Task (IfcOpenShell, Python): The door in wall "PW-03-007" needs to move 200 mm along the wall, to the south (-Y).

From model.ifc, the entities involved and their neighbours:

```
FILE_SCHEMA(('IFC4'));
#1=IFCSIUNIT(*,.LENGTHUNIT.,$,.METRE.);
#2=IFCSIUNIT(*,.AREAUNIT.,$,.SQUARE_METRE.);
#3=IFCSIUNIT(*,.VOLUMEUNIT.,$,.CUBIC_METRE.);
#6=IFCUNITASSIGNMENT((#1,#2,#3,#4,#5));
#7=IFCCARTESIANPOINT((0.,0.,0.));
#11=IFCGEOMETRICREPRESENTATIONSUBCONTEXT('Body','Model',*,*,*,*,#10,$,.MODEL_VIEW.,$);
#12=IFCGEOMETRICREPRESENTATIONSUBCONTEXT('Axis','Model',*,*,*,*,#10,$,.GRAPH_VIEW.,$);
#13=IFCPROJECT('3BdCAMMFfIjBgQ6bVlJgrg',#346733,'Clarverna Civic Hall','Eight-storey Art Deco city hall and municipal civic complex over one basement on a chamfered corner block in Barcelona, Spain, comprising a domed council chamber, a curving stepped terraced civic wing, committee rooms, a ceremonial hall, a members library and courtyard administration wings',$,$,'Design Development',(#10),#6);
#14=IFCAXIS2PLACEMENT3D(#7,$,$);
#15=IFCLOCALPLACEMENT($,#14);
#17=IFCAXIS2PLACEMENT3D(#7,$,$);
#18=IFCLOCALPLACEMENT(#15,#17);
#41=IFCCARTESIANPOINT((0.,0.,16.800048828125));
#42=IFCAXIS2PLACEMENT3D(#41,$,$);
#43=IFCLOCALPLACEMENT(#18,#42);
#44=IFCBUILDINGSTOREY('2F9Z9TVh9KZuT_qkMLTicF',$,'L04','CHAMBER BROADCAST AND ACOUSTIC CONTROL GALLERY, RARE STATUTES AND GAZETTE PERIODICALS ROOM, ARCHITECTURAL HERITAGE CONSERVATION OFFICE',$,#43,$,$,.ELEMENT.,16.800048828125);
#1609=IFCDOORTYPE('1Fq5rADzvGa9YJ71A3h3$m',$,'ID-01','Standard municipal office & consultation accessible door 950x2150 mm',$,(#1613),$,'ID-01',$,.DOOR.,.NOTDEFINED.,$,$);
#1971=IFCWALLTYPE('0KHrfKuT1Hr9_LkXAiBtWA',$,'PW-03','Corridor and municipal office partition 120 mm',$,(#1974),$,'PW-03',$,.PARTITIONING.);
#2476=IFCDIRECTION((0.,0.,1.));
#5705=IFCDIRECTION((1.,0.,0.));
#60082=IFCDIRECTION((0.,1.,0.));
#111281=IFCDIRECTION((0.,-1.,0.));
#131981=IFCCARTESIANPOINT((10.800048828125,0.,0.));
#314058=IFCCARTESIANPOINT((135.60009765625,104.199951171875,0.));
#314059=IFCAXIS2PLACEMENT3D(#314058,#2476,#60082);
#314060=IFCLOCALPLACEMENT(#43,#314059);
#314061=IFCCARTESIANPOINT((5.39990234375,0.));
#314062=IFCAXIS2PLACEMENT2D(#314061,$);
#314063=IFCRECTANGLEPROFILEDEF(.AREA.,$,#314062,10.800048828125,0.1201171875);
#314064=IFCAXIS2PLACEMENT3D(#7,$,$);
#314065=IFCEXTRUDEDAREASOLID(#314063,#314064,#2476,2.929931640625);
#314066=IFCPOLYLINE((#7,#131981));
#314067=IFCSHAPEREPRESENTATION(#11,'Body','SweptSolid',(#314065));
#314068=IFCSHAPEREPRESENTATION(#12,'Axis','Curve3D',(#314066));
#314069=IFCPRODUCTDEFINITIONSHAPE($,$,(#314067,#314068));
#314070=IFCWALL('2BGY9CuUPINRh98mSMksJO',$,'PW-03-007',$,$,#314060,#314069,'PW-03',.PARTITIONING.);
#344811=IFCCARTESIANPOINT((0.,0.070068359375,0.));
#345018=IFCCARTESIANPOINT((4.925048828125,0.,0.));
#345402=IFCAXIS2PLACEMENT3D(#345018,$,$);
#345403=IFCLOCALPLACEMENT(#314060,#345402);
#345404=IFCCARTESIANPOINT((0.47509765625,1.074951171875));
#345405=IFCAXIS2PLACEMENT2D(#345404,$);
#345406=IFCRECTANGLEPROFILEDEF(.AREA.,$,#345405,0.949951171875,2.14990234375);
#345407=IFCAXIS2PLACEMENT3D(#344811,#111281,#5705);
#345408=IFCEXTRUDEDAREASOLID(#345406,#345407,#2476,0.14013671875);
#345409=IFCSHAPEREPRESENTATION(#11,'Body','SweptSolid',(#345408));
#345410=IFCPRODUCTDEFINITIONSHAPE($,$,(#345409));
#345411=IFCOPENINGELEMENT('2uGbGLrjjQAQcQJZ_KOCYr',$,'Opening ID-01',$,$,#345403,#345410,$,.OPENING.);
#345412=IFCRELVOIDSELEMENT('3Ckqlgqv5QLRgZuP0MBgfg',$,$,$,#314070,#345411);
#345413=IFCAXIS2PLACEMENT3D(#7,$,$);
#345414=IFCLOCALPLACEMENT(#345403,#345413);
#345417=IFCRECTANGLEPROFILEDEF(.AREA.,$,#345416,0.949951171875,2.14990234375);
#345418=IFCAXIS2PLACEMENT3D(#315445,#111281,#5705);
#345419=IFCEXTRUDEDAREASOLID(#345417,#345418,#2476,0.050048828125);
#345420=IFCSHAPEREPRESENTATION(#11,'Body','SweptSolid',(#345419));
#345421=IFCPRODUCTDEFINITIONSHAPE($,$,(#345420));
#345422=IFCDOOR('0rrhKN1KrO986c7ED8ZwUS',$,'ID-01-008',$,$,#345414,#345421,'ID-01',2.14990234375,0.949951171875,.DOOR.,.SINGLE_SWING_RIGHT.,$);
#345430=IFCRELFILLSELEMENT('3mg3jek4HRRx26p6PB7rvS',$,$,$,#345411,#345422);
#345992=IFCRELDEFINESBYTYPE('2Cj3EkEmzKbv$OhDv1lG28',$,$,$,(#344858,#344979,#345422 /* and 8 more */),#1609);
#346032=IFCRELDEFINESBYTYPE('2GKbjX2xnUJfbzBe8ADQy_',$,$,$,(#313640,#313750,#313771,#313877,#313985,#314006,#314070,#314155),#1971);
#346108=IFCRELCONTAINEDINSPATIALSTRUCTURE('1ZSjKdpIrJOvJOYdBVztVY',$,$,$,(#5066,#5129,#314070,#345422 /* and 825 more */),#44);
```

```python
import ifcopenshell
import ifcopenshell.api.geometry
import ifcopenshell.util.placement

model = ifcopenshell.open("model.ifc")

door = model.by_id(345422)
opening = door.FillsVoids[0].RelatingOpeningElement
wall = opening.VoidsElements[0].RelatingBuildingElement

wall_matrix = ifcopenshell.util.placement.get_local_placement(wall.ObjectPlacement)
shift = wall_matrix[:3, 0] * -0.2
before = ifcopenshell.util.placement.get_local_placement(door.ObjectPlacement)[:3, 3].copy()

# The door is placed relative to its opening, so it follows when the opening moves.
matrix = ifcopenshell.util.placement.get_local_placement(opening.ObjectPlacement)
matrix[:3, 3] += shift
ifcopenshell.api.geometry.edit_object_placement(
    model, product=opening, matrix=matrix, is_si=False, should_transform_children=True
)

after = ifcopenshell.util.placement.get_local_placement(door.ObjectPlacement)[:3, 3]
print("door moved by", (after - before).round(3) + 0.0)

model.write("model_v2.ifc")
```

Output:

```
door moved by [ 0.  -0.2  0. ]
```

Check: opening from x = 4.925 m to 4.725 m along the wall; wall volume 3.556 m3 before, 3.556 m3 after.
